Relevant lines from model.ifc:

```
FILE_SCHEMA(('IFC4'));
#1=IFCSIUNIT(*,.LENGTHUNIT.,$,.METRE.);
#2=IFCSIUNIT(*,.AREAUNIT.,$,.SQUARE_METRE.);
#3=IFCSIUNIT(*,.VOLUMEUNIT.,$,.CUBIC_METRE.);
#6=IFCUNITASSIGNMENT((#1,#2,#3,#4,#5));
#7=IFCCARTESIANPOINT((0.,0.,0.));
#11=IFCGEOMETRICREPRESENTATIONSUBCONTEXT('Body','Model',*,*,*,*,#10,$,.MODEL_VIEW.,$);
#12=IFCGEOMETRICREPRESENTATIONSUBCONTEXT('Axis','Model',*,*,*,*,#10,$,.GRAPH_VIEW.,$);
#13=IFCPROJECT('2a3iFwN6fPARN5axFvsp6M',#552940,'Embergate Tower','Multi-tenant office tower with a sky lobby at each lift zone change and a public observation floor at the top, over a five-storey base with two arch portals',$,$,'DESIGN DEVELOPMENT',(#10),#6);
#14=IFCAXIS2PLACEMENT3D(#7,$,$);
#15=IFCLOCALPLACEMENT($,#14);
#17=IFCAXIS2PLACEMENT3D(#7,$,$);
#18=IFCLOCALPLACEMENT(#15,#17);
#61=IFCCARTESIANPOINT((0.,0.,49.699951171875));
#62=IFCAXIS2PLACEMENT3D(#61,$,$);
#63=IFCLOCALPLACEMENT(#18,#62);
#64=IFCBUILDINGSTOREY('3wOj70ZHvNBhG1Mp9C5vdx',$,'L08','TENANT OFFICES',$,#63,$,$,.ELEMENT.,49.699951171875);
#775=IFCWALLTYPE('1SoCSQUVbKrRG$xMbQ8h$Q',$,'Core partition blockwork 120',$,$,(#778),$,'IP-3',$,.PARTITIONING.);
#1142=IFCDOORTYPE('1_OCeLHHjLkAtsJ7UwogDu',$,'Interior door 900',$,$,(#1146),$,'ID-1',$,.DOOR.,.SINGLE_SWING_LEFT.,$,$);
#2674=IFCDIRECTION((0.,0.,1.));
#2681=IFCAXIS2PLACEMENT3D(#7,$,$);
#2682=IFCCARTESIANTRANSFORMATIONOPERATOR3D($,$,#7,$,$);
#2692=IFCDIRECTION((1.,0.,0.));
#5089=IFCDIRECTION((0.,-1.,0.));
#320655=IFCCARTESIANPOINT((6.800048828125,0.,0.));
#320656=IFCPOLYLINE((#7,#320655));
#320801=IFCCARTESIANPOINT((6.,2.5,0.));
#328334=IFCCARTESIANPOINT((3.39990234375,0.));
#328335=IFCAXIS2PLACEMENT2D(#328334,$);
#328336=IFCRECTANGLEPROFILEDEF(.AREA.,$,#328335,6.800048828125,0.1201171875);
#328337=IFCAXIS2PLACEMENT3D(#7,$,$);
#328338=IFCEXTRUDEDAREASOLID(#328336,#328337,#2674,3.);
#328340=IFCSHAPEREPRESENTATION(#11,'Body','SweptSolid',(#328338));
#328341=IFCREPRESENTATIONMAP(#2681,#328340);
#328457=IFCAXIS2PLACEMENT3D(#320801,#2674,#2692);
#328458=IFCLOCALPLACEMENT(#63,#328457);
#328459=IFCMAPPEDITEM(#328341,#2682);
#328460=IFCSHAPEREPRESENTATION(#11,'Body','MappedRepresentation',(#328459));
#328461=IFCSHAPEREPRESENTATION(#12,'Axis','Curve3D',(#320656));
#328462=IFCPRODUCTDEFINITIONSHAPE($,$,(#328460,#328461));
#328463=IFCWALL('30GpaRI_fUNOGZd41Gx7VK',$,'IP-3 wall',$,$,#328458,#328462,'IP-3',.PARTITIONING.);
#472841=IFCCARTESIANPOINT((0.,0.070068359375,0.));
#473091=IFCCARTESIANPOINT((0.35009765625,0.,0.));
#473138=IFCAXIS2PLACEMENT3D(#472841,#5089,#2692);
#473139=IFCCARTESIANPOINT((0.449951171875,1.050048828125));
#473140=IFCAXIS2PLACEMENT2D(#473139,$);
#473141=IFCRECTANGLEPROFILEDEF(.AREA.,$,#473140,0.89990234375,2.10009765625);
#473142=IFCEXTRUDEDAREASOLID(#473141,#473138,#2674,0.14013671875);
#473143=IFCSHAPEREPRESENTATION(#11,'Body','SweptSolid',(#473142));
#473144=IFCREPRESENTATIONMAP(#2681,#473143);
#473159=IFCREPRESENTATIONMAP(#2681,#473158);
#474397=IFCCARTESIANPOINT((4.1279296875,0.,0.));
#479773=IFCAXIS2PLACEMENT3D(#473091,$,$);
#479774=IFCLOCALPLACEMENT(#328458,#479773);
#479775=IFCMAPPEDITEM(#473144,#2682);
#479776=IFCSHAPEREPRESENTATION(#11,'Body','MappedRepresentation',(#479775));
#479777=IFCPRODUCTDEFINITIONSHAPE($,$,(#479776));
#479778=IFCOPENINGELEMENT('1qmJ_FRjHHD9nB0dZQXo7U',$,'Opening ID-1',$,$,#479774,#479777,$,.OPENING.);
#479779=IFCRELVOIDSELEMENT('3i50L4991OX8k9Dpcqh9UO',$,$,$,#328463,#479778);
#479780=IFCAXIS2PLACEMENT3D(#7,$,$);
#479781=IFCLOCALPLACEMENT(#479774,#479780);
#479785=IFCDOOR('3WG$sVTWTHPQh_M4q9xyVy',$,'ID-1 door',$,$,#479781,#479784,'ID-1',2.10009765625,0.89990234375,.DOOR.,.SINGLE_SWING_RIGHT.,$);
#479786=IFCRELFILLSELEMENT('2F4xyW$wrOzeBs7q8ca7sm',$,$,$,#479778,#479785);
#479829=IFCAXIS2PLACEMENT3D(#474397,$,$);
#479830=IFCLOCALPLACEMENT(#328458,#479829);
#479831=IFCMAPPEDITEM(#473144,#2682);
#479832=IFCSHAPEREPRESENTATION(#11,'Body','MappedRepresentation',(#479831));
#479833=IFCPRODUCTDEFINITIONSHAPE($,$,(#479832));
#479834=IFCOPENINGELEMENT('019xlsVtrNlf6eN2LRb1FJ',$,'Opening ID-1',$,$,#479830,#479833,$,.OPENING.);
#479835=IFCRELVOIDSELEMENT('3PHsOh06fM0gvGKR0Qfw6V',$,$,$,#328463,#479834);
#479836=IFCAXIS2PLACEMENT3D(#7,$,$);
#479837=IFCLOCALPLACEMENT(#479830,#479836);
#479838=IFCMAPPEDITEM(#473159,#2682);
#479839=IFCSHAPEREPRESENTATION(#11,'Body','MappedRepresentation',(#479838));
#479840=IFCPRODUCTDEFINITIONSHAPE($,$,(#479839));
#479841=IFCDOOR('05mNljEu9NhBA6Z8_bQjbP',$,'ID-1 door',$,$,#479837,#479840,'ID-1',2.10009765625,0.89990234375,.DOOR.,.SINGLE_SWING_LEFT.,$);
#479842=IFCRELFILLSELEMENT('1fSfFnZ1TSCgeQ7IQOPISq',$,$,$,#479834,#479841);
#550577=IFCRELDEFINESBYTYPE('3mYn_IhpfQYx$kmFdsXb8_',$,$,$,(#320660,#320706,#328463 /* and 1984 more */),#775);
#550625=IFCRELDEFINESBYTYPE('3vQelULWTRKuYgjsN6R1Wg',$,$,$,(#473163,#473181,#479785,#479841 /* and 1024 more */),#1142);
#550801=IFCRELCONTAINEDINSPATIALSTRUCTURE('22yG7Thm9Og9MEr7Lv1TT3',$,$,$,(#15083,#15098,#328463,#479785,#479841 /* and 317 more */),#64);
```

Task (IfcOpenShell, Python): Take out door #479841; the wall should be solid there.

```python
import ifcopenshell
import ifcopenshell.api.feature
import ifcopenshell.api.root
import ifcopenshell.geom
import ifcopenshell.util.shape

model = ifcopenshell.open("model.ifc")
settings = ifcopenshell.geom.settings()


def volume(element):
    """Net volume in cubic metres, openings subtracted."""
    shape = ifcopenshell.geom.create_shape(settings, element)
    return ifcopenshell.util.shape.get_volume(shape.geometry)


door = model.by_id(479841)
opening = door.FillsVoids[0].RelatingOpeningElement
wall = opening.VoidsElements[0].RelatingBuildingElement
before = volume(wall)

ifcopenshell.api.root.remove_product(model, product=door)
ifcopenshell.api.feature.remove_feature(model, feature=opening)

after = volume(wall)

print(f"wall volume {before:.3f} -> {after:.3f} m3")

model.write("model-out.ifc")
```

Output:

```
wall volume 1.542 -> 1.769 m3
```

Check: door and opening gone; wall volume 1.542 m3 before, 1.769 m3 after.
